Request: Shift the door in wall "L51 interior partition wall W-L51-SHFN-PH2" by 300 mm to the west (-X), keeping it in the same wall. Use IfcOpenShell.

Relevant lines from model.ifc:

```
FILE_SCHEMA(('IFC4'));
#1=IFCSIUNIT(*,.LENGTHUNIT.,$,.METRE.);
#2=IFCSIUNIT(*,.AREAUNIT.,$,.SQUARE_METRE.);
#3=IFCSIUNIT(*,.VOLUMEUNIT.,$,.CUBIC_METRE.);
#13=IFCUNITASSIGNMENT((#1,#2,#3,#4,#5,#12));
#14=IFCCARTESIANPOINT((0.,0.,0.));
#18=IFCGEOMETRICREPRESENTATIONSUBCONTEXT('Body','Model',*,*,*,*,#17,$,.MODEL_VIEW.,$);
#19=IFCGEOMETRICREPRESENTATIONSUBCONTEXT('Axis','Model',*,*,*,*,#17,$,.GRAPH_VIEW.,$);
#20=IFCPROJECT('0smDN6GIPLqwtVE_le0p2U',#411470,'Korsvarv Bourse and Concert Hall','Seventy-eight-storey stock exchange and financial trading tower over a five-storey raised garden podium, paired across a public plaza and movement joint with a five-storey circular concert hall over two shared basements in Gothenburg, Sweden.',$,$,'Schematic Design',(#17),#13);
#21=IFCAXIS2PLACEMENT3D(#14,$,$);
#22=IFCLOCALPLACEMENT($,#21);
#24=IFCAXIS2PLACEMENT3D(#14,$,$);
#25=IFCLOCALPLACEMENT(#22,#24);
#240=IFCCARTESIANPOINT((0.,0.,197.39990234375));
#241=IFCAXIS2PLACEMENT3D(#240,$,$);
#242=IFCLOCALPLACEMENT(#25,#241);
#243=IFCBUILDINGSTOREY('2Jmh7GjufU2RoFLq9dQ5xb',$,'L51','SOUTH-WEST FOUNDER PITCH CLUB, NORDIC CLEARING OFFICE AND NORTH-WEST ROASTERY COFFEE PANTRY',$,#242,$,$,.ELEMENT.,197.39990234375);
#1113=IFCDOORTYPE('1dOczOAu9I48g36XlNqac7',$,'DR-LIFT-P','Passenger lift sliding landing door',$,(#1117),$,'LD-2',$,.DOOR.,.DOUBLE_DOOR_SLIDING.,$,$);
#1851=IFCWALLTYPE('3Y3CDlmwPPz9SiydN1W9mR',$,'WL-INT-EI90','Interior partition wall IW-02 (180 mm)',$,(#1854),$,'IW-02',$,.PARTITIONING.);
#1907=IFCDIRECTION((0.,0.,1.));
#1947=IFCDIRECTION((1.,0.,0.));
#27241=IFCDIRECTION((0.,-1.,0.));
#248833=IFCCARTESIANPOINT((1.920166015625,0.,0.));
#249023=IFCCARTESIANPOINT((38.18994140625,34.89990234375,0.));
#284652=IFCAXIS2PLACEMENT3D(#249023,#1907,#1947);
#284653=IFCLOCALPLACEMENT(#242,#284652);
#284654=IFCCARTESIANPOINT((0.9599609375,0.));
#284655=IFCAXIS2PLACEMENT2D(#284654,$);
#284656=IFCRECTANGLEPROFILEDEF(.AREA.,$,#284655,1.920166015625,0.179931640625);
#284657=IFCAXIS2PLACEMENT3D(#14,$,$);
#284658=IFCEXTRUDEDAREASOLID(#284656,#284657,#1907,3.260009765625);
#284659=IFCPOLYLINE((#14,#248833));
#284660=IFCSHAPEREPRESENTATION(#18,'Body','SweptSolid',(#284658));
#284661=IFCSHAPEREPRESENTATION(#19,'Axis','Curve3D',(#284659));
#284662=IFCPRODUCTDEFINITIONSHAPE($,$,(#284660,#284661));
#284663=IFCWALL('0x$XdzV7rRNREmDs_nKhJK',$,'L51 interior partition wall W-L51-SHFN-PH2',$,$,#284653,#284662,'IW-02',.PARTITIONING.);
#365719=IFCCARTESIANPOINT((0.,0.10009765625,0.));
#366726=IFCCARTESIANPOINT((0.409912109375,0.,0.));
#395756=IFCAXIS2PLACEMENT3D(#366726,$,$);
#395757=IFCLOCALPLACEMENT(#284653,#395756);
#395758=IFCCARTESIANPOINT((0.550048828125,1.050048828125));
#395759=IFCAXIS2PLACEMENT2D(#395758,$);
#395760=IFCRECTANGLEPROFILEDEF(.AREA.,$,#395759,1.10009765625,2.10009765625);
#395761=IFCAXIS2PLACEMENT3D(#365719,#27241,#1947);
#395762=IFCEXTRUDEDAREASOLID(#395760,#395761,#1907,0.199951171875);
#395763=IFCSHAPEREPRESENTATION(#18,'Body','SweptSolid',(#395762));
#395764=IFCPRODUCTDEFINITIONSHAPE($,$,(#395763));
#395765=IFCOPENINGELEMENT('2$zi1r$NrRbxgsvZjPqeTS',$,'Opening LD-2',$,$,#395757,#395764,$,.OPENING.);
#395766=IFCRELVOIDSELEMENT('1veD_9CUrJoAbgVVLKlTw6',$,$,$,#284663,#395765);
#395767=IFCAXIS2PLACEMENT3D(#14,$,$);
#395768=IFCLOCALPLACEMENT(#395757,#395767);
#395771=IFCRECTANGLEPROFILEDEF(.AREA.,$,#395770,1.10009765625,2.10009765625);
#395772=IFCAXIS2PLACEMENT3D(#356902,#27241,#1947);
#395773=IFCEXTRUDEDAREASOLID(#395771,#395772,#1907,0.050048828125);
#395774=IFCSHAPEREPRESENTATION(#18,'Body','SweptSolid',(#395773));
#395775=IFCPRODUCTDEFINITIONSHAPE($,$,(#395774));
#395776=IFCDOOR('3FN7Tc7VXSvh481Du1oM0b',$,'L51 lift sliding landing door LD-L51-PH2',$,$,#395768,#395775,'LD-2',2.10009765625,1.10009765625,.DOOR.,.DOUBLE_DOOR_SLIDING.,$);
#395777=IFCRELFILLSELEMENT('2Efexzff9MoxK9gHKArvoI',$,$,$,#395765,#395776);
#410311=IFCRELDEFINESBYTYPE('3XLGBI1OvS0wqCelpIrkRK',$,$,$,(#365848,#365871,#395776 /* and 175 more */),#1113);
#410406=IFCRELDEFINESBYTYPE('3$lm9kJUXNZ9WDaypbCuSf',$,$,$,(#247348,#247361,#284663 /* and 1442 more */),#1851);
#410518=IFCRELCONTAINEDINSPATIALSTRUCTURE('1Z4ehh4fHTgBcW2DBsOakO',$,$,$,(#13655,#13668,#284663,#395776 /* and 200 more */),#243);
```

```python
import ifcopenshell
import ifcopenshell.api.geometry
import ifcopenshell.util.placement

model = ifcopenshell.open("model.ifc")

door = model.by_guid("3FN7Tc7VXSvh481Du1oM0b")
opening = door.FillsVoids[0].RelatingOpeningElement
wall = opening.VoidsElements[0].RelatingBuildingElement

wall_matrix = ifcopenshell.util.placement.get_local_placement(wall.ObjectPlacement)
shift = wall_matrix[:3, 0] * -0.3
before = ifcopenshell.util.placement.get_local_placement(door.ObjectPlacement)[:3, 3].copy()

# The door is placed relative to its opening, so it follows when the opening moves.
matrix = ifcopenshell.util.placement.get_local_placement(opening.ObjectPlacement)
matrix[:3, 3] += shift
ifcopenshell.api.geometry.edit_object_placement(
    model, product=opening, matrix=matrix, is_si=False, should_transform_children=True
)

after = ifcopenshell.util.placement.get_local_placement(door.ObjectPlacement)[:3, 3]
print("door moved by", (after - before).round(3) + 0.0)

model.write("model-out.ifc")
```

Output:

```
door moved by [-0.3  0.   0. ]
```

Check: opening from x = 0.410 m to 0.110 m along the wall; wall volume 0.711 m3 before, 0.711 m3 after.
